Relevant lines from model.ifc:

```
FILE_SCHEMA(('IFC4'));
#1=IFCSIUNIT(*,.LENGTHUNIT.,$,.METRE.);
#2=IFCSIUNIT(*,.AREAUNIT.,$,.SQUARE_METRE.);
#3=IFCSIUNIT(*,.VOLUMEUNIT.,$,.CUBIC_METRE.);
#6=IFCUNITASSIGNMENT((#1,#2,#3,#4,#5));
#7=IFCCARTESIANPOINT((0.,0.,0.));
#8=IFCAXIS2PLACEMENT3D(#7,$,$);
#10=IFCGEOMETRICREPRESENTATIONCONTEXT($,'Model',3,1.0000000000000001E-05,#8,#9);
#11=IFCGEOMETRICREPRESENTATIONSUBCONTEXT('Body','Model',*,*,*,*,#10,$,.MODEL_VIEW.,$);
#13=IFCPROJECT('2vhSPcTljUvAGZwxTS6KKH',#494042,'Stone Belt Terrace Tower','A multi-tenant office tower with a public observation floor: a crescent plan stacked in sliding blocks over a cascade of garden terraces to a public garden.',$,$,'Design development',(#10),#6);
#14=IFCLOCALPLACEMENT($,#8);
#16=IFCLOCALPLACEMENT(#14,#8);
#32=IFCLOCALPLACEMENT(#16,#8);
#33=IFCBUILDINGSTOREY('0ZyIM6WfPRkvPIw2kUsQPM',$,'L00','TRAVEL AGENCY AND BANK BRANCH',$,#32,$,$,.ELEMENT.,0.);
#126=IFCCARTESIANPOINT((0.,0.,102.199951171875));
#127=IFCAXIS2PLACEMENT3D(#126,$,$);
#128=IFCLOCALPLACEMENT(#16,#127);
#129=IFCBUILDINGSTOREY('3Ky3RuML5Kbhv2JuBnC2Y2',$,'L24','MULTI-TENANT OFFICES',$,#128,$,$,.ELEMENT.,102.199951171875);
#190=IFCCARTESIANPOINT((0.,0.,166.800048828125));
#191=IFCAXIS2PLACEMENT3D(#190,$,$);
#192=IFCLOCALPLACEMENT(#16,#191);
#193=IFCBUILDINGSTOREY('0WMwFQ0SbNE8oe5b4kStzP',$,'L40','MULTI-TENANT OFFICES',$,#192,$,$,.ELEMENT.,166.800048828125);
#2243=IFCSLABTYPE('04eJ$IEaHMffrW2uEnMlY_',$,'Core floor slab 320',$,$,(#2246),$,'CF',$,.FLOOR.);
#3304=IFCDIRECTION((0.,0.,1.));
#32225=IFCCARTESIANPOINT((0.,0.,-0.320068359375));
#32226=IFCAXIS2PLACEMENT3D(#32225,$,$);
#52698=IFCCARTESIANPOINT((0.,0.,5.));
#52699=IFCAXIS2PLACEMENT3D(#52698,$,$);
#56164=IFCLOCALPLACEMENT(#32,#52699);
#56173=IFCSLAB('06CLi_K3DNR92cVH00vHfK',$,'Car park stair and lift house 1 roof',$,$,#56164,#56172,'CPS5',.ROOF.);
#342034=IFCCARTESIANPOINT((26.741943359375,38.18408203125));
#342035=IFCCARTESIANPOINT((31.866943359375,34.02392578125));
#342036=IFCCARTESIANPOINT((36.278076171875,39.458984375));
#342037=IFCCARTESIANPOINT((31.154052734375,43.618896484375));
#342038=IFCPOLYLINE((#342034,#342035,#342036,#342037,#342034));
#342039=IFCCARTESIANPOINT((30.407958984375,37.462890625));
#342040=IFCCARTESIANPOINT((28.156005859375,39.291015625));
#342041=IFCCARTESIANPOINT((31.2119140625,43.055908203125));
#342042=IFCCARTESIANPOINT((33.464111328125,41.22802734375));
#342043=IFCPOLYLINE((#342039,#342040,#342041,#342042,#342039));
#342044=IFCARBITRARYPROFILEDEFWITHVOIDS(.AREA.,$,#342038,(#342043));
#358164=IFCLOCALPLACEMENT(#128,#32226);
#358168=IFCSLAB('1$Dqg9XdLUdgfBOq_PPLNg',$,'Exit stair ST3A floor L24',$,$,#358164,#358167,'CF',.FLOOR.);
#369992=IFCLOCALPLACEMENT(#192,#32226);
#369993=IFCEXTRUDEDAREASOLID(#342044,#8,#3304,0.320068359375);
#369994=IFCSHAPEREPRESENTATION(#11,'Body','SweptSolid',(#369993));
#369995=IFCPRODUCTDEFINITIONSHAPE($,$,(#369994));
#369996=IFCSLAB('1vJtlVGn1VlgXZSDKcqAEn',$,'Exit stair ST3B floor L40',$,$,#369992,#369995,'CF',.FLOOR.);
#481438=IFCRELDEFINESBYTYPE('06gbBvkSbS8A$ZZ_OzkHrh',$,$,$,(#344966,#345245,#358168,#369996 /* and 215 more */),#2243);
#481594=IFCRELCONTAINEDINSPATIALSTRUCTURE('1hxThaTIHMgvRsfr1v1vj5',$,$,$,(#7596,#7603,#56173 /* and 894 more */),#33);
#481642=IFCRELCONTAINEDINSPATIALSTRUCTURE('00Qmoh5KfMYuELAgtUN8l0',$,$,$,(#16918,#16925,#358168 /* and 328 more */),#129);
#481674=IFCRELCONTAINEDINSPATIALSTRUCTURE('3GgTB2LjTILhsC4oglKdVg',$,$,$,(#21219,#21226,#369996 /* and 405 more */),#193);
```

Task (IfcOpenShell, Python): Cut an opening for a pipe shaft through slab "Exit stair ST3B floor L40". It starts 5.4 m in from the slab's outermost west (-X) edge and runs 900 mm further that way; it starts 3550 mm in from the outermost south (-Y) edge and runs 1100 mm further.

```python
import numpy as np
import ifcopenshell
import ifcopenshell.api.feature
import ifcopenshell.api.geometry
import ifcopenshell.api.root
import ifcopenshell.geom
import ifcopenshell.util.placement
import ifcopenshell.util.representation
import ifcopenshell.util.shape
import ifcopenshell.util.unit

model = ifcopenshell.open("model.ifc")
unit_scale = ifcopenshell.util.unit.calculate_unit_scale(model)
settings = ifcopenshell.geom.settings()


def volume(element):
    """Net volume in cubic metres, openings subtracted."""
    shape = ifcopenshell.geom.create_shape(settings, element)
    return ifcopenshell.util.shape.get_volume(shape.geometry)


slab = model.by_guid("1vJtlVGn1VlgXZSDKcqAEn")
before = volume(slab)

# Extent in the slab's own axes, in metres. The edges named are its -X and -Y sides.
slab_shape = ifcopenshell.geom.create_shape(settings, slab)
vertices = ifcopenshell.util.shape.get_vertices(slab_shape.geometry)
x_min, y_min, bottom = vertices.min(axis=0)
top = vertices[:, 2].max()

opening = ifcopenshell.api.root.create_entity(model, ifc_class="IfcOpeningElement", name="Pipe shaft opening", predefined_type="OPENING")
context = ifcopenshell.util.representation.get_context(model, "Model", "Body", "MODEL_VIEW")
width, depth = 0.9, 1.1
outline = [(0.0, 0.0), (width, 0.0), (width, depth), (0.0, depth), (0.0, 0.0)]
# Overshoot both faces by 50 mm so the cut is clean.
shape = ifcopenshell.api.geometry.add_slab_representation(
    model, context=context, depth=top - bottom + 0.1, polyline=outline
)
ifcopenshell.api.geometry.assign_representation(model, product=opening, representation=shape)

matrix = ifcopenshell.util.placement.get_local_placement(slab.ObjectPlacement)
matrix[:, 3] = matrix @ np.append(np.array([x_min + 5.4, y_min + 3.55, bottom - 0.05]) / unit_scale, 1.0)
ifcopenshell.api.geometry.edit_object_placement(model, product=opening, matrix=matrix, is_si=False)
ifcopenshell.api.feature.add_feature(model, feature=opening, element=slab)

after = volume(slab)

print(f"slab volume {before:.3f} -> {after:.3f} m3")

model.write("model-out.ifc")
```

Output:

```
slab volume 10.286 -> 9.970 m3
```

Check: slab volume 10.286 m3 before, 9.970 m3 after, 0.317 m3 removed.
